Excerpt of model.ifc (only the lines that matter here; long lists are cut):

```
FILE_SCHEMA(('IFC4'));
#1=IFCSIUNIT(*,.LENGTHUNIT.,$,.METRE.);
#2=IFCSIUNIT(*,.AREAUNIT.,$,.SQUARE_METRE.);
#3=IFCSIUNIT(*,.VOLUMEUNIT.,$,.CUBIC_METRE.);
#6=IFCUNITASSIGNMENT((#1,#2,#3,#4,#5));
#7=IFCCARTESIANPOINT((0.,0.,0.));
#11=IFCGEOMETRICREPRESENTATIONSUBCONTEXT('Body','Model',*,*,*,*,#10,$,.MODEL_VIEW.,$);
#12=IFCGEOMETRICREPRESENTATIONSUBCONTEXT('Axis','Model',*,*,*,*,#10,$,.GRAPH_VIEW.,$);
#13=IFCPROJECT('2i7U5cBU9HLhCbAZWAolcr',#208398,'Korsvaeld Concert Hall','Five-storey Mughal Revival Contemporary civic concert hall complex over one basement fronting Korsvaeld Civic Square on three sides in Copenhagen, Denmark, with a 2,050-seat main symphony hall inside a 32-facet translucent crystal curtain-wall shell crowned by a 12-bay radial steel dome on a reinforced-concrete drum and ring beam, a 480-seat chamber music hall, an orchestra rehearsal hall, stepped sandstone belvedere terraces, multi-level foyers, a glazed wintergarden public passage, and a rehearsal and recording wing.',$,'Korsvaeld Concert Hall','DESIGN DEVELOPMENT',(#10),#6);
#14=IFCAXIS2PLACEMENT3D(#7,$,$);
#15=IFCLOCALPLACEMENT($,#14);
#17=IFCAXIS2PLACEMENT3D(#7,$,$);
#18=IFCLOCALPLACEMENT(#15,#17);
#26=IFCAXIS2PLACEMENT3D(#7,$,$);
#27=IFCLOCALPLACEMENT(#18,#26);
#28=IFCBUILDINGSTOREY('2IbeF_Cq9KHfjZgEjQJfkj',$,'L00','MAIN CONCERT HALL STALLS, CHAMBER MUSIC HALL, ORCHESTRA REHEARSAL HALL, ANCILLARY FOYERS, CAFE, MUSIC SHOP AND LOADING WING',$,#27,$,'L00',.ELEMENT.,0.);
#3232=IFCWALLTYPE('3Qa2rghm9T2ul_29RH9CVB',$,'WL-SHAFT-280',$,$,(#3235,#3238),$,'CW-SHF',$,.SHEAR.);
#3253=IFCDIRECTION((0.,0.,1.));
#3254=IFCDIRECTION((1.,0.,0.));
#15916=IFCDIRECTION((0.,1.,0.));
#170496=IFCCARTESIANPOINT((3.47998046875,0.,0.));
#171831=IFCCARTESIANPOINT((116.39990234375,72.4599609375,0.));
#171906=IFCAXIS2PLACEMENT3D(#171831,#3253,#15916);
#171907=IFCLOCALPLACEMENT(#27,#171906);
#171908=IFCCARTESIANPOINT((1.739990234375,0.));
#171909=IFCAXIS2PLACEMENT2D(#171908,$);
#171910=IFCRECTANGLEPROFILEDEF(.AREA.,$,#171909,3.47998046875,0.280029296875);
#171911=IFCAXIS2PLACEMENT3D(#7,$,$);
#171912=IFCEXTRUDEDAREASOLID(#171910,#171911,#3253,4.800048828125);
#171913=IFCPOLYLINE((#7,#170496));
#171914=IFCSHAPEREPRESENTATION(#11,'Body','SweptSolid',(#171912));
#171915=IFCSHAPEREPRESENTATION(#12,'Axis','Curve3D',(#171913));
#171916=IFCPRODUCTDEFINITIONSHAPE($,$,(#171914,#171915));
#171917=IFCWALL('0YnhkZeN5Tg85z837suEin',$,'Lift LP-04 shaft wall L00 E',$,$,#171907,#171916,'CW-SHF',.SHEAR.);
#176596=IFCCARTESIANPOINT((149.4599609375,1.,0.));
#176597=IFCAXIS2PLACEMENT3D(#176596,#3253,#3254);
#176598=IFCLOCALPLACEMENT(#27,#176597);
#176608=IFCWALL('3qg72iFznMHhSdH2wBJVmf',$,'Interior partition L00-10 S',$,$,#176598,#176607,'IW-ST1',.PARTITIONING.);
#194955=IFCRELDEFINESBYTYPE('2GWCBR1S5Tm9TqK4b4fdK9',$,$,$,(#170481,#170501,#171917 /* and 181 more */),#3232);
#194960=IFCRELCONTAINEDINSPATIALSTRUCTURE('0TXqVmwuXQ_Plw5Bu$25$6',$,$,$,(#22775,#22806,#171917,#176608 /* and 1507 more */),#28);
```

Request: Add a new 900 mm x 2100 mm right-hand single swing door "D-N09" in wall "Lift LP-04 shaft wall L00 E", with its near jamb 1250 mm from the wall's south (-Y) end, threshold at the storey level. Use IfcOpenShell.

```python
import numpy as np
import ifcopenshell
import ifcopenshell.api.feature
import ifcopenshell.api.geometry
import ifcopenshell.api.root
import ifcopenshell.api.spatial
import ifcopenshell.geom
import ifcopenshell.util.element
import ifcopenshell.util.placement
import ifcopenshell.util.representation
import ifcopenshell.util.shape
import ifcopenshell.util.unit

model = ifcopenshell.open("model.ifc")
unit_scale = ifcopenshell.util.unit.calculate_unit_scale(model)
settings = ifcopenshell.geom.settings()


def volume(element):
    """Net volume in cubic metres, openings subtracted."""
    shape = ifcopenshell.geom.create_shape(settings, element)
    return ifcopenshell.util.shape.get_volume(shape.geometry)


wall = model.by_id(171917)
storey = ifcopenshell.util.element.get_container(wall, ifc_class="IfcBuildingStorey")
context = ifcopenshell.util.representation.get_context(model, "Model", "Body", "MODEL_VIEW")
before = volume(wall)

width, height, from_end, sill = 0.9, 2.1, 1.25, 0.0  # metres

# The wall runs along its own X axis, and the end named is its -X end.
wall_shape = ifcopenshell.geom.create_shape(settings, wall)
x, y, z = ifcopenshell.util.shape.get_vertices(wall_shape.geometry).T
start = x.min() + from_end
face, thickness = float(y.min()), float(y.max() - y.min())
wall_matrix = ifcopenshell.util.placement.get_local_placement(wall.ObjectPlacement)
level = ifcopenshell.util.placement.get_local_placement(storey.ObjectPlacement)[2, 3]


def in_wall(x, y):
    """Placement at x, y metres in the wall's axes, at sill height."""
    matrix = wall_matrix.copy()
    matrix[:, 3] = wall_matrix @ np.array([x / unit_scale, y / unit_scale, 0.0, 1.0])
    matrix[2, 3] = level + sill / unit_scale
    return matrix


# Opening: a box that overshoots both wall faces by 50 mm.
opening = ifcopenshell.api.root.create_entity(model, ifc_class="IfcOpeningElement", predefined_type="OPENING")
box = ifcopenshell.api.geometry.add_wall_representation(
    model, context=context, length=width, height=height, thickness=thickness + 0.1
)
ifcopenshell.api.geometry.assign_representation(model, product=opening, representation=box)
ifcopenshell.api.geometry.edit_object_placement(model, product=opening, matrix=in_wall(start, face - 0.05), is_si=False)
ifcopenshell.api.feature.add_feature(model, feature=opening, element=wall)

door = ifcopenshell.api.root.create_entity(model, ifc_class="IfcDoor", name="D-N09", predefined_type="DOOR")
door.OverallWidth, door.OverallHeight = width / unit_scale, height / unit_scale
door.OperationType = "SINGLE_SWING_RIGHT"
body = ifcopenshell.api.geometry.add_door_representation(
    model,
    context=context,
    overall_width=door.OverallWidth,
    overall_height=door.OverallHeight,
    operation_type="SINGLE_SWING_RIGHT",
    lining_properties={"LiningDepth": thickness / unit_scale, "ThresholdDepth": thickness / unit_scale},
)
ifcopenshell.api.geometry.assign_representation(model, product=door, representation=body)
ifcopenshell.api.spatial.assign_container(model, products=[door], relating_structure=storey)
ifcopenshell.api.feature.add_filling(model, opening=opening, element=door)

# The lining spans the wall, so the door starts at the wall face.
ifcopenshell.api.geometry.edit_object_placement(model, product=door, matrix=in_wall(start, face), is_si=False)

after = volume(wall)

print(f"wall volume {before:.3f} -> {after:.3f} m3")

model.write("model_rev.ifc")
```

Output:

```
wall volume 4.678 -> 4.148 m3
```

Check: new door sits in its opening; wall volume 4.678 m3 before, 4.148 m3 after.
